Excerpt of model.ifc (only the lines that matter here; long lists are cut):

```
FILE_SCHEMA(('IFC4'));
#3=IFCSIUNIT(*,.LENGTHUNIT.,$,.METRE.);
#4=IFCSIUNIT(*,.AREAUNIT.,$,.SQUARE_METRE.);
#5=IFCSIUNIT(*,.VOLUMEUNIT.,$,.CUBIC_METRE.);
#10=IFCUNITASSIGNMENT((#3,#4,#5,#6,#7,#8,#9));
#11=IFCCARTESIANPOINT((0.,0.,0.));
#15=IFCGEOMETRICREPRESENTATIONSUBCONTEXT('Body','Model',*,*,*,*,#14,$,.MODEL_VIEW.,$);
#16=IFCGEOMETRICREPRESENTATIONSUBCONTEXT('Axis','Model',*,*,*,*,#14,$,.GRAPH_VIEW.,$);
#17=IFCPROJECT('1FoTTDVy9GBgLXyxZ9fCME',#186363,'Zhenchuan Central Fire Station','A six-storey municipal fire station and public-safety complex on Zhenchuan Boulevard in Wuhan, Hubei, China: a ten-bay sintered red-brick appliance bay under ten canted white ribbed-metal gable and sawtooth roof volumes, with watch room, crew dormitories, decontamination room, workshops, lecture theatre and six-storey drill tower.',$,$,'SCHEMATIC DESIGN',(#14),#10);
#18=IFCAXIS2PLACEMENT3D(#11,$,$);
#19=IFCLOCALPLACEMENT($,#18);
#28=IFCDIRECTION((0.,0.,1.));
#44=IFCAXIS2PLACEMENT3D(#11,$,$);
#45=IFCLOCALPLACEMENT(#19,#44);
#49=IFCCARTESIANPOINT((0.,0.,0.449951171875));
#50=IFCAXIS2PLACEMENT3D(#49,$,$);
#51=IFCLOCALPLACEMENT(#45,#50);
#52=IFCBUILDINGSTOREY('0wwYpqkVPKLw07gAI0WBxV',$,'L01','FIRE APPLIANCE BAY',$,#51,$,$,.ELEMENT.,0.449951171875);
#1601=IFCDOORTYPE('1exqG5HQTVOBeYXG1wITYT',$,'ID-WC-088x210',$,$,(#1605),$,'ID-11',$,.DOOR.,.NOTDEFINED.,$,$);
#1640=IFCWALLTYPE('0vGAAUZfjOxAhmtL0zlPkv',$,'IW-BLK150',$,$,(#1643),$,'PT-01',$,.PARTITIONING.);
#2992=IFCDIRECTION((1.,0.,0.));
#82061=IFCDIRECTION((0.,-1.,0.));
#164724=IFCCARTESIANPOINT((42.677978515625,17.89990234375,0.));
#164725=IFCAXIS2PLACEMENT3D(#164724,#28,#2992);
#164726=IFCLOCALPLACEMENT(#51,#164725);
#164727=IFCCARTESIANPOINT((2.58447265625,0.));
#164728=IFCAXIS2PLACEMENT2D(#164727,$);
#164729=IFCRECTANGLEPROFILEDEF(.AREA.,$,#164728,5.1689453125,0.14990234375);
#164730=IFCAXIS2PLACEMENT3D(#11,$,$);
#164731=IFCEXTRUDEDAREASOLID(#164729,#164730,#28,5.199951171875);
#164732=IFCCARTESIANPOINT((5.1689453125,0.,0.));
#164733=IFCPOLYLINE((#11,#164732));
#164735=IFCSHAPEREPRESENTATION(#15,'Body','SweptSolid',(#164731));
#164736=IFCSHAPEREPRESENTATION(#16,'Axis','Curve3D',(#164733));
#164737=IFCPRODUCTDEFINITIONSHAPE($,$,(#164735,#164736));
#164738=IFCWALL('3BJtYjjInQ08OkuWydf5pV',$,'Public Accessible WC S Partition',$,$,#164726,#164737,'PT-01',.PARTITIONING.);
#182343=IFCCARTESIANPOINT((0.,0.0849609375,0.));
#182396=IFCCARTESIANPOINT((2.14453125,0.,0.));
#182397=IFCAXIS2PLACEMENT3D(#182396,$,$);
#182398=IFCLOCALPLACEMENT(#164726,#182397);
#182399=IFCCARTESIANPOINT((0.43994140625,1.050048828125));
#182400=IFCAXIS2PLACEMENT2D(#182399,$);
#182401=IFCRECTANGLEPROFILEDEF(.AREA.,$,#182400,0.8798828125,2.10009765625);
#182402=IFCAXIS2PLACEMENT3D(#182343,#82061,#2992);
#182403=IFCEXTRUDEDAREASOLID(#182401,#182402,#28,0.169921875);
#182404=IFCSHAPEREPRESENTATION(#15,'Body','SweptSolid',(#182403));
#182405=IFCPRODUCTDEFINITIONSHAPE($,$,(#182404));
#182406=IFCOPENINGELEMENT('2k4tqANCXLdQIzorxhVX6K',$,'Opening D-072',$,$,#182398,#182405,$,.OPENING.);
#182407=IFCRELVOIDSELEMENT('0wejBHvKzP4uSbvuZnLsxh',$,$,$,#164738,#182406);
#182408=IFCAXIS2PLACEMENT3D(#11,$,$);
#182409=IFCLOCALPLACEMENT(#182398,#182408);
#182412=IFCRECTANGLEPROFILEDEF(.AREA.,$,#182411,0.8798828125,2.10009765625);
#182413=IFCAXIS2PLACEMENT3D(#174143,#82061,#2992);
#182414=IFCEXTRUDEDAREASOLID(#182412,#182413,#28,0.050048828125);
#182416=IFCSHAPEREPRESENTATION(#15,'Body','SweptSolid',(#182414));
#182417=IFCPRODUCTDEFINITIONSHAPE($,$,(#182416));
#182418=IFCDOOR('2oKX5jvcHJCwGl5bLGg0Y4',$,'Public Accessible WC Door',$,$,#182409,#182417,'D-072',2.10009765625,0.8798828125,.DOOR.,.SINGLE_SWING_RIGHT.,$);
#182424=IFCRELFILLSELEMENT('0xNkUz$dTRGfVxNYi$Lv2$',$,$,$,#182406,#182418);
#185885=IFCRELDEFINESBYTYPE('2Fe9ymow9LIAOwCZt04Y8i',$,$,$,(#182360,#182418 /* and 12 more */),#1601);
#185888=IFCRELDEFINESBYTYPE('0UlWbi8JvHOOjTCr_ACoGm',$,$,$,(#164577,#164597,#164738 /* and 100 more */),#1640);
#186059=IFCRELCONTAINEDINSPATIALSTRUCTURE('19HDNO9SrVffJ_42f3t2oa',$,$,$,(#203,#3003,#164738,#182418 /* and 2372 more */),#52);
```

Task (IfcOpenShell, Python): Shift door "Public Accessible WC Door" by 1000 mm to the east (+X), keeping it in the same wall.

```python
import ifcopenshell
import ifcopenshell.api.geometry
import ifcopenshell.util.placement

model = ifcopenshell.open("model.ifc")

door = model.by_id(182418)
opening = door.FillsVoids[0].RelatingOpeningElement
wall = opening.VoidsElements[0].RelatingBuildingElement

wall_matrix = ifcopenshell.util.placement.get_local_placement(wall.ObjectPlacement)
shift = wall_matrix[:3, 0] * 1.0
before = ifcopenshell.util.placement.get_local_placement(door.ObjectPlacement)[:3, 3].copy()

# The door is placed relative to its opening, so it follows when the opening moves.
matrix = ifcopenshell.util.placement.get_local_placement(opening.ObjectPlacement)
matrix[:3, 3] += shift
ifcopenshell.api.geometry.edit_object_placement(
    model, product=opening, matrix=matrix, is_si=False, should_transform_children=True
)

after = ifcopenshell.util.placement.get_local_placement(door.ObjectPlacement)[:3, 3]
print("door moved by", (after - before).round(3) + 0.0)

model.write("model_updated.ifc")
```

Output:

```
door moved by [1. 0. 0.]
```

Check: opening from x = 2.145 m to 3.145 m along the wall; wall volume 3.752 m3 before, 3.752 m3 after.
